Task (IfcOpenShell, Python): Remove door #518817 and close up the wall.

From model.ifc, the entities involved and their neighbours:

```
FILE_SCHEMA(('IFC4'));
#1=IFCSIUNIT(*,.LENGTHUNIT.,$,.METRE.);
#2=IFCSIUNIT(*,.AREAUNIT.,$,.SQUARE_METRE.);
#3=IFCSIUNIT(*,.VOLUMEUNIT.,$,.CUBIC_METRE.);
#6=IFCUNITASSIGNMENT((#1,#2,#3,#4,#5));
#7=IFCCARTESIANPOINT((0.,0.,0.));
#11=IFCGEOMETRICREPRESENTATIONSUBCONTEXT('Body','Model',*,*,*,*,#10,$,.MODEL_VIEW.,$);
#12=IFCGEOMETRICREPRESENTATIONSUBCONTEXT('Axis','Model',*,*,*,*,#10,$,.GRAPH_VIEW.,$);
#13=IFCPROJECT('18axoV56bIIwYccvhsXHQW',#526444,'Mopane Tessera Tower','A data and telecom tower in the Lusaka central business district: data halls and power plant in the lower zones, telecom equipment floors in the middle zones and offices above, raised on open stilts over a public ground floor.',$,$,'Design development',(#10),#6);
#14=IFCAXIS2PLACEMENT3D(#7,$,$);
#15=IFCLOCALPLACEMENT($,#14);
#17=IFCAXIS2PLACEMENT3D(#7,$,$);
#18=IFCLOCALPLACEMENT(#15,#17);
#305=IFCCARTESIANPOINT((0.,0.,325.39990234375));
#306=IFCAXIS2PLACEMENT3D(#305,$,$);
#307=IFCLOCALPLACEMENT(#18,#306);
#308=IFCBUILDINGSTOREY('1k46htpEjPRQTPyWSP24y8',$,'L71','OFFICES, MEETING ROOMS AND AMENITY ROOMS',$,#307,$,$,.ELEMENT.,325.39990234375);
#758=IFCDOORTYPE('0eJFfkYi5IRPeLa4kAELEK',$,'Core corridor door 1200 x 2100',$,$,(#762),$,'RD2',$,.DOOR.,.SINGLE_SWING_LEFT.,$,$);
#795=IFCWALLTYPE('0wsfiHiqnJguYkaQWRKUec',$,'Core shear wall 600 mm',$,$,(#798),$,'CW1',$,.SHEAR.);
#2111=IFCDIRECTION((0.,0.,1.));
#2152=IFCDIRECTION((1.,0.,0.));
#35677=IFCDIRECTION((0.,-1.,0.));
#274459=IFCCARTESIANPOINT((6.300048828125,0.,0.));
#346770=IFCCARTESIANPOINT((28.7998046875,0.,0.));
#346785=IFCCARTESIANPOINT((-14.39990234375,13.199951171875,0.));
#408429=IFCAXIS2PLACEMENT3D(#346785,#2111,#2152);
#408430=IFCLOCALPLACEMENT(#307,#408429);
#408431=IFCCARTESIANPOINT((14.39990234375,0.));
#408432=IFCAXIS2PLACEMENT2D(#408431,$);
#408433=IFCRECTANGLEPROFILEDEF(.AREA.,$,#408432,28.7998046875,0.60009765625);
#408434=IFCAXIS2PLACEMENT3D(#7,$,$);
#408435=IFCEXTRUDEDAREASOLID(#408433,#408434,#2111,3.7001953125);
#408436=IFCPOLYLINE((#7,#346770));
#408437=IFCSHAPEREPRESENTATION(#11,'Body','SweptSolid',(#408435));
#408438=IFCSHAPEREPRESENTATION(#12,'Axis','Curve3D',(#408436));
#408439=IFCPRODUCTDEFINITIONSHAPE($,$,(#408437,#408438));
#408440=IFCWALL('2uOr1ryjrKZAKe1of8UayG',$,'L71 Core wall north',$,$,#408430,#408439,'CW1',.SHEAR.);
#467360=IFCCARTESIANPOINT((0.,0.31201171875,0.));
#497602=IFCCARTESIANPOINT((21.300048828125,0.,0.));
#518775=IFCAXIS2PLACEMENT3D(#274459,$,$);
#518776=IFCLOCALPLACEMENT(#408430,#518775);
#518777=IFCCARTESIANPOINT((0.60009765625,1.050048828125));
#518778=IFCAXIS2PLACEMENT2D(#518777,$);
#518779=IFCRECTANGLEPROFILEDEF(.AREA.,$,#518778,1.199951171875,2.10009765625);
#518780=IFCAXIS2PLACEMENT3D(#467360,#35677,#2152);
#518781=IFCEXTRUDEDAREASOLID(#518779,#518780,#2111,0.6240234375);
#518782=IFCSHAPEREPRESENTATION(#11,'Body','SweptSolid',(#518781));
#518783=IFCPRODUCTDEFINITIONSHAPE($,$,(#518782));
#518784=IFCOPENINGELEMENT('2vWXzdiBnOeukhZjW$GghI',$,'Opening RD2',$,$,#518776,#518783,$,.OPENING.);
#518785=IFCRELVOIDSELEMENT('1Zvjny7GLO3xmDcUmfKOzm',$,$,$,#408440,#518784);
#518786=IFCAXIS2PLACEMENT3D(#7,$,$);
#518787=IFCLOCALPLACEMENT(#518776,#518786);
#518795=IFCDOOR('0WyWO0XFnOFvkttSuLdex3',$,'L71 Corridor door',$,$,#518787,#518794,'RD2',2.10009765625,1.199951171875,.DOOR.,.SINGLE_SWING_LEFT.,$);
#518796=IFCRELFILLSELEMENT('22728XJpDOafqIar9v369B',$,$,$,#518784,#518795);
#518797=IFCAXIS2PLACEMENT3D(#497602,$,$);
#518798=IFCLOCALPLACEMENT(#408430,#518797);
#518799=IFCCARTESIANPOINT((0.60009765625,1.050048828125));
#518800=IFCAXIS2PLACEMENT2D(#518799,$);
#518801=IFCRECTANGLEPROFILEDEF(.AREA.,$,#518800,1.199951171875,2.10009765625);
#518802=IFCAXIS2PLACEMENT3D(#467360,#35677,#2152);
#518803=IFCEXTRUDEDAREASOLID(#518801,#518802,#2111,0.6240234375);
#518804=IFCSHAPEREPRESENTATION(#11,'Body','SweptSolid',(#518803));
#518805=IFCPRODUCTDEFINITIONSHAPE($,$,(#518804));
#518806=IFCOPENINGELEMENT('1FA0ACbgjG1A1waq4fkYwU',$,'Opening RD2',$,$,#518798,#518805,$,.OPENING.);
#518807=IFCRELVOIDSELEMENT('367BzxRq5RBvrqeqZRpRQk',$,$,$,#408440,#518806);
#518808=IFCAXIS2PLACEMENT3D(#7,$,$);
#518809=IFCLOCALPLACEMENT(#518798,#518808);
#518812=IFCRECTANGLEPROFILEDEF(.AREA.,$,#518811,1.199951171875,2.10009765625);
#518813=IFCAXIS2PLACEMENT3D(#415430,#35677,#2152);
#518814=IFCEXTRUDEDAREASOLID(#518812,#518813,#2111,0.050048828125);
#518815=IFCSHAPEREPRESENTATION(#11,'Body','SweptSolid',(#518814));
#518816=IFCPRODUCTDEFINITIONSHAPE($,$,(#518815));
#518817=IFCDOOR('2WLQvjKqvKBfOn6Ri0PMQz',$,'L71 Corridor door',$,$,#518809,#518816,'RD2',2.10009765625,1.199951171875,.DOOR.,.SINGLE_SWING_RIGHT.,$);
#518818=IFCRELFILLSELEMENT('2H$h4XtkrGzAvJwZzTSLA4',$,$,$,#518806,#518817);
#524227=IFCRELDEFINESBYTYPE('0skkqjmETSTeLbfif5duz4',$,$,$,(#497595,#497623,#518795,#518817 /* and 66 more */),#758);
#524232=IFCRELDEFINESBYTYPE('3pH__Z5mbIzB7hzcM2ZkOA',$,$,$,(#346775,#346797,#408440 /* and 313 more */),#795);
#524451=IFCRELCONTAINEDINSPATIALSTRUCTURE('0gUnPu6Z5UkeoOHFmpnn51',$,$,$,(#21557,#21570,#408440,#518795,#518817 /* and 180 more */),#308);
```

```python
import ifcopenshell
import ifcopenshell.api.feature
import ifcopenshell.api.root
import ifcopenshell.geom
import ifcopenshell.util.shape

model = ifcopenshell.open("model.ifc")
settings = ifcopenshell.geom.settings()


def volume(element):
    """Net volume in cubic metres, openings subtracted."""
    shape = ifcopenshell.geom.create_shape(settings, element)
    return ifcopenshell.util.shape.get_volume(shape.geometry)


door = model.by_guid("2WLQvjKqvKBfOn6Ri0PMQz")
opening = door.FillsVoids[0].RelatingOpeningElement
wall = opening.VoidsElements[0].RelatingBuildingElement
before = volume(wall)

ifcopenshell.api.root.remove_product(model, product=door)
ifcopenshell.api.feature.remove_feature(model, feature=opening)

after = volume(wall)

print(f"wall volume {before:.3f} -> {after:.3f} m3")

model.write("model_v2.ifc")
```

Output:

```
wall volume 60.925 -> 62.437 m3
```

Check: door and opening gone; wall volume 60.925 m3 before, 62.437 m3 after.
